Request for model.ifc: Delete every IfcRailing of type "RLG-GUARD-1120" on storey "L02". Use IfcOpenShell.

First a look at what the model holds.

```python
import ifcopenshell
import ifcopenshell.util.element

model = ifcopenshell.open("model.ifc")
print(model.schema)
storey = next(s for s in model.by_type("IfcBuildingStorey") if s.Name == "L02")
railings = [e for e in ifcopenshell.util.element.get_decomposition(storey) if e.is_a("IfcRailing")]
seen = {}
for e in railings:
    element_type = ifcopenshell.util.element.get_type(e)
    name = element_type.Name if element_type not in (None, e) else None
    seen[name] = seen.get(name, 0) + 1
for name, count in sorted(seen.items(), key=str):
    print(count, "x", name)
```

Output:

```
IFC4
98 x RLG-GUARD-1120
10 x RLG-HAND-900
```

```python
import ifcopenshell
import ifcopenshell.api.root
import ifcopenshell.util.element

model = ifcopenshell.open("model.ifc")

storey = next(s for s in model.by_type("IfcBuildingStorey") if s.Name == "L02")
railings = [e for e in ifcopenshell.util.element.get_decomposition(storey) if e.is_a("IfcRailing")]
targets = [e for e in railings if (t := ifcopenshell.util.element.get_type(e)) not in (None, e) and t.Name == "RLG-GUARD-1120"]

for e in targets:
    ifcopenshell.api.root.remove_product(model, product=e)
print(len(targets), "removed")

model.write("model_updated.ifc")
```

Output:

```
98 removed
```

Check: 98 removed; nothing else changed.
